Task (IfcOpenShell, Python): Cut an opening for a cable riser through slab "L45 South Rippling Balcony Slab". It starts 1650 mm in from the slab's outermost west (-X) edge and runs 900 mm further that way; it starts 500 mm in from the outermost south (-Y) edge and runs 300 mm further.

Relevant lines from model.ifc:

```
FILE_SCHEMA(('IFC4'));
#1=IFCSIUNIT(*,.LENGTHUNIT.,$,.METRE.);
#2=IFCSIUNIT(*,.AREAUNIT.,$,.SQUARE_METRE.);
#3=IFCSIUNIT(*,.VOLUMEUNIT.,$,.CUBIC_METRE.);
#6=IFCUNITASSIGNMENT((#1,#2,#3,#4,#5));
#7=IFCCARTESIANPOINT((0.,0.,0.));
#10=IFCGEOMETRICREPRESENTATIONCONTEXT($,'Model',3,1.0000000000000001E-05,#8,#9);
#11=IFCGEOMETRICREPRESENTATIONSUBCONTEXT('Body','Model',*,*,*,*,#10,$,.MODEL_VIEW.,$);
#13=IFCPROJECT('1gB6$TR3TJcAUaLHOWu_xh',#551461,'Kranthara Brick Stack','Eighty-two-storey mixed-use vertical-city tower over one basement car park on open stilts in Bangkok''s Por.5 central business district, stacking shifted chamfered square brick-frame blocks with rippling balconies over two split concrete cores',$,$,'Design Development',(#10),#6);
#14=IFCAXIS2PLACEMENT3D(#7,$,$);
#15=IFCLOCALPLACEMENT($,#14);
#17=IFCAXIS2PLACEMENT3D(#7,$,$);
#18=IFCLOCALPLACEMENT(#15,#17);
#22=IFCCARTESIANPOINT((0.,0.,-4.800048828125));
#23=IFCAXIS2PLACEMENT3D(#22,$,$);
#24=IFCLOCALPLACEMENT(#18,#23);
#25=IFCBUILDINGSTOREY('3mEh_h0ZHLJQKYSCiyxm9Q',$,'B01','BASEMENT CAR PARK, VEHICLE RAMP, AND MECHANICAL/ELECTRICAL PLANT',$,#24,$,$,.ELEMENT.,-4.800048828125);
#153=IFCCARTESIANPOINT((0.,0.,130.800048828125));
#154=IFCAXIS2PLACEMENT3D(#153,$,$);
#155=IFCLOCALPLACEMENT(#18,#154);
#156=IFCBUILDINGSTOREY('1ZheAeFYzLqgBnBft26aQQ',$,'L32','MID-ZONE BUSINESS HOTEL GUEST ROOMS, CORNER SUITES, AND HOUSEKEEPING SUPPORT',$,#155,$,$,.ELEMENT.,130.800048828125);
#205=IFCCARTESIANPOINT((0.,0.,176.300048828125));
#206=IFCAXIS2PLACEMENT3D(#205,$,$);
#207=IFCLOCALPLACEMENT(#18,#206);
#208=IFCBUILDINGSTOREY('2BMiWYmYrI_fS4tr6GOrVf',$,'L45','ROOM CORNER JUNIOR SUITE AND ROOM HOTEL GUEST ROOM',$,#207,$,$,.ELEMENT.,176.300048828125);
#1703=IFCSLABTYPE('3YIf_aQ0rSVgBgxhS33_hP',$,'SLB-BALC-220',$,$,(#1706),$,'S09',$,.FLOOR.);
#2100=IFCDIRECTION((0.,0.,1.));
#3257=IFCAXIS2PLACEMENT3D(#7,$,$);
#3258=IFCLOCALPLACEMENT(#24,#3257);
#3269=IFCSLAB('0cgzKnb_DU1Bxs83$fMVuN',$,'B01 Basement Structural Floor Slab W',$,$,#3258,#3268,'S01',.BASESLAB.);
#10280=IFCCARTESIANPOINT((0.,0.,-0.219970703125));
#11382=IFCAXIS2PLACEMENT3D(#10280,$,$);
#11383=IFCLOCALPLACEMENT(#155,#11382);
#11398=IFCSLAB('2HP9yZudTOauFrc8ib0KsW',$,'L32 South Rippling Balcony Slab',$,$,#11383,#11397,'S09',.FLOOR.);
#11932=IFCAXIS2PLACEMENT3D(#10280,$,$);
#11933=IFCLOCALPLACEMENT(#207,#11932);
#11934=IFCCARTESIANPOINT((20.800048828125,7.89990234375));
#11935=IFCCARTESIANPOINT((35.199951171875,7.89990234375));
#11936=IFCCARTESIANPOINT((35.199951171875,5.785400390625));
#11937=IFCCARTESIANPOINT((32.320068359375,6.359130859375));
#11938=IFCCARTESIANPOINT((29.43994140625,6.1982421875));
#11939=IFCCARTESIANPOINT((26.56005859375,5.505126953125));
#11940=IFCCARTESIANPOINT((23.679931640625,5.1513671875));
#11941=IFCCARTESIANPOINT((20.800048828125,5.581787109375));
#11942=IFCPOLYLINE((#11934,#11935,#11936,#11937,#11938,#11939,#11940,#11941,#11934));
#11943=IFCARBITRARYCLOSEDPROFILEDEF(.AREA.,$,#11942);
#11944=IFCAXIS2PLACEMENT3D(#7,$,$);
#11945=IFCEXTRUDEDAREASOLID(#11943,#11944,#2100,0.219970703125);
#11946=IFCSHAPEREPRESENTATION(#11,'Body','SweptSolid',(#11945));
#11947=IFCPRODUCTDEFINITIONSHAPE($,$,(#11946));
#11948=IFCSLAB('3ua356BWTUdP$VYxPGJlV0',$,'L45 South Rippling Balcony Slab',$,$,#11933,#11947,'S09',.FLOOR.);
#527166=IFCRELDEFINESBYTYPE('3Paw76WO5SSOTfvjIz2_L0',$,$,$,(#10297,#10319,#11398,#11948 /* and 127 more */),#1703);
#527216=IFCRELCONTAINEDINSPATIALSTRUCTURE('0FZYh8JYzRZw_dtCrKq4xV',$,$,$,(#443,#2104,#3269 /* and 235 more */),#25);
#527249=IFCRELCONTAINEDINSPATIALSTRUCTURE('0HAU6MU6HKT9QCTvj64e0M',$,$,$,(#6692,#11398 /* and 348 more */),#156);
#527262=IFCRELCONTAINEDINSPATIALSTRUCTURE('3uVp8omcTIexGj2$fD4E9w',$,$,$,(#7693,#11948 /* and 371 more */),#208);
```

```python
import numpy as np
import ifcopenshell
import ifcopenshell.api.feature
import ifcopenshell.api.geometry
import ifcopenshell.api.root
import ifcopenshell.geom
import ifcopenshell.util.placement
import ifcopenshell.util.representation
import ifcopenshell.util.shape
import ifcopenshell.util.unit

model = ifcopenshell.open("model.ifc")
unit_scale = ifcopenshell.util.unit.calculate_unit_scale(model)
settings = ifcopenshell.geom.settings()


def volume(element):
    """Net volume in cubic metres, openings subtracted."""
    shape = ifcopenshell.geom.create_shape(settings, element)
    return ifcopenshell.util.shape.get_volume(shape.geometry)


slab = model.by_guid("3ua356BWTUdP$VYxPGJlV0")
before = volume(slab)

# Extent in the slab's own axes, in metres. The edges named are its -X and -Y sides.
slab_shape = ifcopenshell.geom.create_shape(settings, slab)
vertices = ifcopenshell.util.shape.get_vertices(slab_shape.geometry)
x_min, y_min, bottom = vertices.min(axis=0)
top = vertices[:, 2].max()

opening = ifcopenshell.api.root.create_entity(model, ifc_class="IfcOpeningElement", name="Cable riser opening", predefined_type="OPENING")
context = ifcopenshell.util.representation.get_context(model, "Model", "Body", "MODEL_VIEW")
width, depth = 0.9, 0.3
outline = [(0.0, 0.0), (width, 0.0), (width, depth), (0.0, depth), (0.0, 0.0)]
# Overshoot both faces by 50 mm so the cut is clean.
shape = ifcopenshell.api.geometry.add_slab_representation(
    model, context=context, depth=top - bottom + 0.1, polyline=outline
)
ifcopenshell.api.geometry.assign_representation(model, product=opening, representation=shape)

matrix = ifcopenshell.util.placement.get_local_placement(slab.ObjectPlacement)
matrix[:, 3] = matrix @ np.append(np.array([x_min + 1.65, y_min + 0.5, bottom - 0.05]) / unit_scale, 1.0)
ifcopenshell.api.geometry.edit_object_placement(model, product=opening, matrix=matrix, is_si=False)
ifcopenshell.api.feature.add_feature(model, feature=opening, element=slab)

after = volume(slab)

print(f"slab volume {before:.3f} -> {after:.3f} m3")

model.write("model-out.ifc")
```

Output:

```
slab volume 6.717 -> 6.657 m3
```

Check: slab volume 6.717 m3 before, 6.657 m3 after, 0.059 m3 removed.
